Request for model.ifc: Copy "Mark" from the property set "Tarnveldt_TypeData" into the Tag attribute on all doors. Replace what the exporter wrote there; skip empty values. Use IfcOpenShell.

First a look at what the model holds.

```python
import ifcopenshell
import ifcopenshell.util.element

model = ifcopenshell.open("model.ifc")
print(model.schema)
doors = model.by_type("IfcDoor")
print(len(doors), "doors")
for e in doors[:8]:
    source = ifcopenshell.util.element.get_pset(e, "Tarnveldt_TypeData", "Mark")
    target = e.Tag
    print(e.id(), repr(source), repr(target), sep=" | ")
```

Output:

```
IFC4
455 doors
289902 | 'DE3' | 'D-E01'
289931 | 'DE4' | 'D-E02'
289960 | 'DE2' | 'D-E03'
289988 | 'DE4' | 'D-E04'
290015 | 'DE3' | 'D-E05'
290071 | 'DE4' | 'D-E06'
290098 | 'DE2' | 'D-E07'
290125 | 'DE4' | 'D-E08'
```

```python
import ifcopenshell
import ifcopenshell.util.element

model = ifcopenshell.open("model.ifc")

count = 0
for e in model.by_type("IfcDoor"):
    value = ifcopenshell.util.element.get_pset(e, "Tarnveldt_TypeData", "Mark")
    current = e.Tag
    if not value or not value.strip() or current == value:
        continue
    e.Tag = value
    count += 1

print(count, "doors updated")

model.write("model_rev.ifc")
```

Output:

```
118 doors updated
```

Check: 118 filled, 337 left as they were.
